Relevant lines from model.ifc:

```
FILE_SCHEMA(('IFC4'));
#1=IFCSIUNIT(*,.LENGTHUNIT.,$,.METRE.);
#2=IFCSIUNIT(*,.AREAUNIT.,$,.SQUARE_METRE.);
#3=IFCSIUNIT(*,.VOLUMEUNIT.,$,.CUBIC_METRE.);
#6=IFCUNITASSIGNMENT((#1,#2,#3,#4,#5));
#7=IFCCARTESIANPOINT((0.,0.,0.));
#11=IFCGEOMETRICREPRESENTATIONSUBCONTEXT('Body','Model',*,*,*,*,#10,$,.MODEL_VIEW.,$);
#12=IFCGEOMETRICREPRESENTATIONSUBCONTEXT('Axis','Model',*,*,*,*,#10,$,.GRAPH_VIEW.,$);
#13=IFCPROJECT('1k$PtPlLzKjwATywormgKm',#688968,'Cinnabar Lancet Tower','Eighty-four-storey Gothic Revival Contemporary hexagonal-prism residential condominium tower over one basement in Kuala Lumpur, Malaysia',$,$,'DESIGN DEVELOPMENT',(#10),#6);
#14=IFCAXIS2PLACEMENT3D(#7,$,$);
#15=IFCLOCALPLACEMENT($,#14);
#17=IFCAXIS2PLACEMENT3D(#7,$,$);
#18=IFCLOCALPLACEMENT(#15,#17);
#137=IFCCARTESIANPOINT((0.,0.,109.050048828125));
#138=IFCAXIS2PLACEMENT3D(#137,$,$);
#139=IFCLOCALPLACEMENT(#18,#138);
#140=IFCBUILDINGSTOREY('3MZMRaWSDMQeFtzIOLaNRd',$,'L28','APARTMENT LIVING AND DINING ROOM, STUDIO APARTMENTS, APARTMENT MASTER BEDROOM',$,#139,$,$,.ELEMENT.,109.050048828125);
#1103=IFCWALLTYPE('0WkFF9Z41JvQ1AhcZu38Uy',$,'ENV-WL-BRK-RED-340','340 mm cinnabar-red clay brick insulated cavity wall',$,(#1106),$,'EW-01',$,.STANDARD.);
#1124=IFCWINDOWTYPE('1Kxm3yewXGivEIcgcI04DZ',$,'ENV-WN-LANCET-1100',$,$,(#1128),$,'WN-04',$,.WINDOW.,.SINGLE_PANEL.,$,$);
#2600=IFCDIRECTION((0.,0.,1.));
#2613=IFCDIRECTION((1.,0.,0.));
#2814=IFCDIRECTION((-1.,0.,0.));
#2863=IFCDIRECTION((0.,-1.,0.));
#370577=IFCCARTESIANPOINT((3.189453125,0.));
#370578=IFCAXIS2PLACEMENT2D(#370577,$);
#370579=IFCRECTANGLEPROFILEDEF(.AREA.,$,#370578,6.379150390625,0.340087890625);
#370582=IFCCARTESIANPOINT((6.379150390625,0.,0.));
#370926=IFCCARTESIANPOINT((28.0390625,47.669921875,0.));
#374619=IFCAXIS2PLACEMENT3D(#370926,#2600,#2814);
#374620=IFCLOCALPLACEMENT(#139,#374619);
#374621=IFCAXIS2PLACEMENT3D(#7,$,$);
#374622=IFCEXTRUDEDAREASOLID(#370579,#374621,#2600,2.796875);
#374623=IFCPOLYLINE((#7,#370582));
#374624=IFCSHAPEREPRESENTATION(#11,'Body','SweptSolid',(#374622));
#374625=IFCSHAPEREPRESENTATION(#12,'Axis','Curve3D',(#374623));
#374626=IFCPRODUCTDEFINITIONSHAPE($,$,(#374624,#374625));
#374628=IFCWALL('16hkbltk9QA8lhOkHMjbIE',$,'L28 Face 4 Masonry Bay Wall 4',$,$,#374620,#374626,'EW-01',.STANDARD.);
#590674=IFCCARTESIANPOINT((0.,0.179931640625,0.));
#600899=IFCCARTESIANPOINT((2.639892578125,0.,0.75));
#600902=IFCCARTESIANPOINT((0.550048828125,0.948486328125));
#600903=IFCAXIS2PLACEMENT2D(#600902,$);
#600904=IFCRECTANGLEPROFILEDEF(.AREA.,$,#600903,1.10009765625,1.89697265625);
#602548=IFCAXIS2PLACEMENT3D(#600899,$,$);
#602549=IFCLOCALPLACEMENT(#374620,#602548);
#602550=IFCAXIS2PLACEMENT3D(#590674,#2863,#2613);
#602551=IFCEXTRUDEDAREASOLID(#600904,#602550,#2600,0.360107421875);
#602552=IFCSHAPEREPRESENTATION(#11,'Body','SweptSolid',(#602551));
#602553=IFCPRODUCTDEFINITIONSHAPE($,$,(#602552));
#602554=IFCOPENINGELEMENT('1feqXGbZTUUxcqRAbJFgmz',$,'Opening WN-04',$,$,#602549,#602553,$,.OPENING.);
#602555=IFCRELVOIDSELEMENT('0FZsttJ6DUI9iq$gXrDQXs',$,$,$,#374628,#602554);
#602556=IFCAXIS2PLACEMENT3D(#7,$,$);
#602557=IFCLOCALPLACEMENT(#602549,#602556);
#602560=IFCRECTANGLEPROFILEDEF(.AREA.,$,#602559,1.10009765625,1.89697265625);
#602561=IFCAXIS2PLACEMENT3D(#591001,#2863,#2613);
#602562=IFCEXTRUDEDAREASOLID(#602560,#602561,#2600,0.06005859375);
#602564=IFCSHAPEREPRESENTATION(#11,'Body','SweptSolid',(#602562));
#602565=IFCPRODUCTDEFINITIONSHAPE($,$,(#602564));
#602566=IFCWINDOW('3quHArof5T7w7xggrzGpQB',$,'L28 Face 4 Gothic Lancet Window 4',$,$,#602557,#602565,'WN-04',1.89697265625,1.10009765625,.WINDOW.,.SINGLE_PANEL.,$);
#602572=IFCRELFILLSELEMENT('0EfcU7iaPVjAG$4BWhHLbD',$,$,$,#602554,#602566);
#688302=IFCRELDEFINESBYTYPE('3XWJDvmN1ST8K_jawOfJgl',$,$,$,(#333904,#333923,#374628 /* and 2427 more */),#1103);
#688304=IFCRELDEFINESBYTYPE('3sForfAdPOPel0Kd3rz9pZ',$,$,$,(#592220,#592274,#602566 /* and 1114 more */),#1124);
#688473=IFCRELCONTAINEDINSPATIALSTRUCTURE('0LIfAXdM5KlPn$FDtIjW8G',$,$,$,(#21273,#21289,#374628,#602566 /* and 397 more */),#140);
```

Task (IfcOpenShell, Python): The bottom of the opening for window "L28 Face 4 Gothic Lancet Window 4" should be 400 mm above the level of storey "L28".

```python
import numpy as np
import ifcopenshell
import ifcopenshell.api.geometry
import ifcopenshell.geom
import ifcopenshell.util.element
import ifcopenshell.util.placement
import ifcopenshell.util.shape
import ifcopenshell.util.unit

model = ifcopenshell.open("model.ifc")
unit_scale = ifcopenshell.util.unit.calculate_unit_scale(model)

window = model.by_guid("3quHArof5T7w7xggrzGpQB")
opening = window.FillsVoids[0].RelatingOpeningElement
storey = ifcopenshell.util.element.get_container(window, ifc_class="IfcBuildingStorey")
level = ifcopenshell.util.placement.get_local_placement(storey.ObjectPlacement)[2, 3]

# The opening's origin need not be at the sill, so measure its lowest point.
shape = ifcopenshell.geom.create_shape(ifcopenshell.geom.settings(), opening)
bottom = ifcopenshell.util.shape.get_shape_bottom_elevation(shape, shape.geometry) / unit_scale
dz = level + 0.4 / unit_scale - bottom

shift = np.array([0.0, 0.0, dz])
# The window is placed relative to its opening, so it follows when the opening moves.
matrix = ifcopenshell.util.placement.get_local_placement(opening.ObjectPlacement)
matrix[:3, 3] += shift
ifcopenshell.api.geometry.edit_object_placement(
    model, product=opening, matrix=matrix, is_si=False, should_transform_children=True
)

print(f"moved by {dz * unit_scale:+.3f} m")

model.write("model_edited.ifc")
```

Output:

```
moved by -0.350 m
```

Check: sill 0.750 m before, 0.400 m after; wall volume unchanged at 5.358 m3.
